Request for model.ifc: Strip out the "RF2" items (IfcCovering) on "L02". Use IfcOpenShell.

First a look at what the model holds.

```python
import ifcopenshell
import ifcopenshell.util.element

model = ifcopenshell.open("model.ifc")
print(model.schema)
storey = next(s for s in model.by_type("IfcBuildingStorey") if s.Name == "L02")
coverings = [e for e in ifcopenshell.util.element.get_decomposition(storey) if e.is_a("IfcCovering")]
seen = {}
for e in coverings:
    element_type = ifcopenshell.util.element.get_type(e)
    name = element_type.Name if element_type not in (None, e) else None
    seen[name] = seen.get(name, 0) + 1
for name, count in sorted(seen.items(), key=str):
    print(count, "x", name)
```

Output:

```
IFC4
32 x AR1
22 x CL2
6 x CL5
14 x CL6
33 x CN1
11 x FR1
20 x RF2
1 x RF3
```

```python
import ifcopenshell
import ifcopenshell.api.root
import ifcopenshell.util.element

model = ifcopenshell.open("model.ifc")

storey = next(s for s in model.by_type("IfcBuildingStorey") if s.Name == "L02")
coverings = [e for e in ifcopenshell.util.element.get_decomposition(storey) if e.is_a("IfcCovering")]
targets = [e for e in coverings if (t := ifcopenshell.util.element.get_type(e)) not in (None, e) and t.Name == "RF2"]

for e in targets:
    ifcopenshell.api.root.remove_product(model, product=e)
print(len(targets), "removed")

model.write("model_v2.ifc")
```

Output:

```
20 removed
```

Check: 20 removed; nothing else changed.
